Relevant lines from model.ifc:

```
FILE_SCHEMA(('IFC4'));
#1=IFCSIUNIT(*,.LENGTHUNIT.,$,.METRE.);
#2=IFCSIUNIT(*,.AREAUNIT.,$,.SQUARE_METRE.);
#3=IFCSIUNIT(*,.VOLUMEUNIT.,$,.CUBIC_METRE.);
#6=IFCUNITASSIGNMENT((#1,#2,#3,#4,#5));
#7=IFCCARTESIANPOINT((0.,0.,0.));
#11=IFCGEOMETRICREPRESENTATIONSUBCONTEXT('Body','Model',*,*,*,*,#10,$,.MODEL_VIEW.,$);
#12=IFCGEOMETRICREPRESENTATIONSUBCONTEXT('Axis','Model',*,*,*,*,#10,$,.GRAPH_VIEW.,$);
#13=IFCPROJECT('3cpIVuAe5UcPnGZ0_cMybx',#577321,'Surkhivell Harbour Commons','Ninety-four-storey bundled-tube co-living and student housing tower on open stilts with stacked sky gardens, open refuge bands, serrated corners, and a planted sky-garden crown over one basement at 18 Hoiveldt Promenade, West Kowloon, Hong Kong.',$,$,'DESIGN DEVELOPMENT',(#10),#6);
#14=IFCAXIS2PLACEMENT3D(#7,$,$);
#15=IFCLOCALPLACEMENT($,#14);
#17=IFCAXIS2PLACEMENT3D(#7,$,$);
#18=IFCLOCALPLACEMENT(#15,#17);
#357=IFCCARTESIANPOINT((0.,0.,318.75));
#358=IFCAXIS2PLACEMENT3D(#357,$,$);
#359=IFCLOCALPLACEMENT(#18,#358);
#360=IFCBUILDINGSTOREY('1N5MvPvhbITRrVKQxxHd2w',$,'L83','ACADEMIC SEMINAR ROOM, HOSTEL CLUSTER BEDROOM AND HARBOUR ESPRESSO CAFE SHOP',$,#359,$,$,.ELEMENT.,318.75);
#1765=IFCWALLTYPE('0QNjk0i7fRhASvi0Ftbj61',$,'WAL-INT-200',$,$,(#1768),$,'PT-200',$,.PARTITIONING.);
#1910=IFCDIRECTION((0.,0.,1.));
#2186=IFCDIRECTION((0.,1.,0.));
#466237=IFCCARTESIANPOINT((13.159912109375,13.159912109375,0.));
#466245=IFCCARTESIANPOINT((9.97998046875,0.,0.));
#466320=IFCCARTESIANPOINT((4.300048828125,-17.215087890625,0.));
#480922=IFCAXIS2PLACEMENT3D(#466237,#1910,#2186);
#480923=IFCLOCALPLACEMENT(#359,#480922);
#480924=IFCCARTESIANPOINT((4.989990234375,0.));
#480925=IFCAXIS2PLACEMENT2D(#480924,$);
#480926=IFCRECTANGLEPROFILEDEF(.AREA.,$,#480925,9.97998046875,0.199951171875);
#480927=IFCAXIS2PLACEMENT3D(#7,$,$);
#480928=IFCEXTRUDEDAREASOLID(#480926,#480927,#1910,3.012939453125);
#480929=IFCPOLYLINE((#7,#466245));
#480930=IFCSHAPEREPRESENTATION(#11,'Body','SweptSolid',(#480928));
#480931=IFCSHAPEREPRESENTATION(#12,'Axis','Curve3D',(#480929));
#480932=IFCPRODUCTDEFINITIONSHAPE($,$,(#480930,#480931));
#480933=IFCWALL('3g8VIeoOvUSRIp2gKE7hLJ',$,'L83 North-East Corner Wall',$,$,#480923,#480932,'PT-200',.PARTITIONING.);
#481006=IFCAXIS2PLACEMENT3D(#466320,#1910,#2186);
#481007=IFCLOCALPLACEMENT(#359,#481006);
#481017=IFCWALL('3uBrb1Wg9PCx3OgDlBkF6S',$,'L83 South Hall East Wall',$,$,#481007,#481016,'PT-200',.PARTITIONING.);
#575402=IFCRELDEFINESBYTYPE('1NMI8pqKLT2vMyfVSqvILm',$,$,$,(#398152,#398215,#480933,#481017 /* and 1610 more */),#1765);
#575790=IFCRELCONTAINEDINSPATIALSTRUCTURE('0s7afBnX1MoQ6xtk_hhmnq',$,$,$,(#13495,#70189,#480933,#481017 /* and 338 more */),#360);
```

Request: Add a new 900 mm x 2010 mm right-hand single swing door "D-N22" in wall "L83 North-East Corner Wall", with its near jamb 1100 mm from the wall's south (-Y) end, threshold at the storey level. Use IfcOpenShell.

```python
import numpy as np
import ifcopenshell
import ifcopenshell.api.feature
import ifcopenshell.api.geometry
import ifcopenshell.api.root
import ifcopenshell.api.spatial
import ifcopenshell.geom
import ifcopenshell.util.element
import ifcopenshell.util.placement
import ifcopenshell.util.representation
import ifcopenshell.util.shape
import ifcopenshell.util.unit

model = ifcopenshell.open("model.ifc")
unit_scale = ifcopenshell.util.unit.calculate_unit_scale(model)
settings = ifcopenshell.geom.settings()


def volume(element):
    """Net volume in cubic metres, openings subtracted."""
    shape = ifcopenshell.geom.create_shape(settings, element)
    return ifcopenshell.util.shape.get_volume(shape.geometry)


wall = model.by_guid("3g8VIeoOvUSRIp2gKE7hLJ")
storey = ifcopenshell.util.element.get_container(wall, ifc_class="IfcBuildingStorey")
context = ifcopenshell.util.representation.get_context(model, "Model", "Body", "MODEL_VIEW")
before = volume(wall)

width, height, from_end, sill = 0.9, 2.01, 1.1, 0.0  # metres

# The wall runs along its own X axis, and the end named is its -X end.
wall_shape = ifcopenshell.geom.create_shape(settings, wall)
x, y, z = ifcopenshell.util.shape.get_vertices(wall_shape.geometry).T
start = x.min() + from_end
face, thickness = float(y.min()), float(y.max() - y.min())
wall_matrix = ifcopenshell.util.placement.get_local_placement(wall.ObjectPlacement)
level = ifcopenshell.util.placement.get_local_placement(storey.ObjectPlacement)[2, 3]


def in_wall(x, y):
    """Placement at x, y metres in the wall's axes, at sill height."""
    matrix = wall_matrix.copy()
    matrix[:, 3] = wall_matrix @ np.array([x / unit_scale, y / unit_scale, 0.0, 1.0])
    matrix[2, 3] = level + sill / unit_scale
    return matrix


# Opening: a box that overshoots both wall faces by 50 mm.
opening = ifcopenshell.api.root.create_entity(model, ifc_class="IfcOpeningElement", predefined_type="OPENING")
box = ifcopenshell.api.geometry.add_wall_representation(
    model, context=context, length=width, height=height, thickness=thickness + 0.1
)
ifcopenshell.api.geometry.assign_representation(model, product=opening, representation=box)
ifcopenshell.api.geometry.edit_object_placement(model, product=opening, matrix=in_wall(start, face - 0.05), is_si=False)
ifcopenshell.api.feature.add_feature(model, feature=opening, element=wall)

door = ifcopenshell.api.root.create_entity(model, ifc_class="IfcDoor", name="D-N22", predefined_type="DOOR")
door.OverallWidth, door.OverallHeight = width / unit_scale, height / unit_scale
door.OperationType = "SINGLE_SWING_RIGHT"
body = ifcopenshell.api.geometry.add_door_representation(
    model,
    context=context,
    overall_width=door.OverallWidth,
    overall_height=door.OverallHeight,
    operation_type="SINGLE_SWING_RIGHT",
    lining_properties={"LiningDepth": thickness / unit_scale, "ThresholdDepth": thickness / unit_scale},
)
ifcopenshell.api.geometry.assign_representation(model, product=door, representation=body)
ifcopenshell.api.spatial.assign_container(model, products=[door], relating_structure=storey)
ifcopenshell.api.feature.add_filling(model, opening=opening, element=door)

# The lining spans the wall, so the door starts at the wall face.
ifcopenshell.api.geometry.edit_object_placement(model, product=door, matrix=in_wall(start, face), is_si=False)

after = volume(wall)

print(f"wall volume {before:.3f} -> {after:.3f} m3")

model.write("model_updated.ifc")
```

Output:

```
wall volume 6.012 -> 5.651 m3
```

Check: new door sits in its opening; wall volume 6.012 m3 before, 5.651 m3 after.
